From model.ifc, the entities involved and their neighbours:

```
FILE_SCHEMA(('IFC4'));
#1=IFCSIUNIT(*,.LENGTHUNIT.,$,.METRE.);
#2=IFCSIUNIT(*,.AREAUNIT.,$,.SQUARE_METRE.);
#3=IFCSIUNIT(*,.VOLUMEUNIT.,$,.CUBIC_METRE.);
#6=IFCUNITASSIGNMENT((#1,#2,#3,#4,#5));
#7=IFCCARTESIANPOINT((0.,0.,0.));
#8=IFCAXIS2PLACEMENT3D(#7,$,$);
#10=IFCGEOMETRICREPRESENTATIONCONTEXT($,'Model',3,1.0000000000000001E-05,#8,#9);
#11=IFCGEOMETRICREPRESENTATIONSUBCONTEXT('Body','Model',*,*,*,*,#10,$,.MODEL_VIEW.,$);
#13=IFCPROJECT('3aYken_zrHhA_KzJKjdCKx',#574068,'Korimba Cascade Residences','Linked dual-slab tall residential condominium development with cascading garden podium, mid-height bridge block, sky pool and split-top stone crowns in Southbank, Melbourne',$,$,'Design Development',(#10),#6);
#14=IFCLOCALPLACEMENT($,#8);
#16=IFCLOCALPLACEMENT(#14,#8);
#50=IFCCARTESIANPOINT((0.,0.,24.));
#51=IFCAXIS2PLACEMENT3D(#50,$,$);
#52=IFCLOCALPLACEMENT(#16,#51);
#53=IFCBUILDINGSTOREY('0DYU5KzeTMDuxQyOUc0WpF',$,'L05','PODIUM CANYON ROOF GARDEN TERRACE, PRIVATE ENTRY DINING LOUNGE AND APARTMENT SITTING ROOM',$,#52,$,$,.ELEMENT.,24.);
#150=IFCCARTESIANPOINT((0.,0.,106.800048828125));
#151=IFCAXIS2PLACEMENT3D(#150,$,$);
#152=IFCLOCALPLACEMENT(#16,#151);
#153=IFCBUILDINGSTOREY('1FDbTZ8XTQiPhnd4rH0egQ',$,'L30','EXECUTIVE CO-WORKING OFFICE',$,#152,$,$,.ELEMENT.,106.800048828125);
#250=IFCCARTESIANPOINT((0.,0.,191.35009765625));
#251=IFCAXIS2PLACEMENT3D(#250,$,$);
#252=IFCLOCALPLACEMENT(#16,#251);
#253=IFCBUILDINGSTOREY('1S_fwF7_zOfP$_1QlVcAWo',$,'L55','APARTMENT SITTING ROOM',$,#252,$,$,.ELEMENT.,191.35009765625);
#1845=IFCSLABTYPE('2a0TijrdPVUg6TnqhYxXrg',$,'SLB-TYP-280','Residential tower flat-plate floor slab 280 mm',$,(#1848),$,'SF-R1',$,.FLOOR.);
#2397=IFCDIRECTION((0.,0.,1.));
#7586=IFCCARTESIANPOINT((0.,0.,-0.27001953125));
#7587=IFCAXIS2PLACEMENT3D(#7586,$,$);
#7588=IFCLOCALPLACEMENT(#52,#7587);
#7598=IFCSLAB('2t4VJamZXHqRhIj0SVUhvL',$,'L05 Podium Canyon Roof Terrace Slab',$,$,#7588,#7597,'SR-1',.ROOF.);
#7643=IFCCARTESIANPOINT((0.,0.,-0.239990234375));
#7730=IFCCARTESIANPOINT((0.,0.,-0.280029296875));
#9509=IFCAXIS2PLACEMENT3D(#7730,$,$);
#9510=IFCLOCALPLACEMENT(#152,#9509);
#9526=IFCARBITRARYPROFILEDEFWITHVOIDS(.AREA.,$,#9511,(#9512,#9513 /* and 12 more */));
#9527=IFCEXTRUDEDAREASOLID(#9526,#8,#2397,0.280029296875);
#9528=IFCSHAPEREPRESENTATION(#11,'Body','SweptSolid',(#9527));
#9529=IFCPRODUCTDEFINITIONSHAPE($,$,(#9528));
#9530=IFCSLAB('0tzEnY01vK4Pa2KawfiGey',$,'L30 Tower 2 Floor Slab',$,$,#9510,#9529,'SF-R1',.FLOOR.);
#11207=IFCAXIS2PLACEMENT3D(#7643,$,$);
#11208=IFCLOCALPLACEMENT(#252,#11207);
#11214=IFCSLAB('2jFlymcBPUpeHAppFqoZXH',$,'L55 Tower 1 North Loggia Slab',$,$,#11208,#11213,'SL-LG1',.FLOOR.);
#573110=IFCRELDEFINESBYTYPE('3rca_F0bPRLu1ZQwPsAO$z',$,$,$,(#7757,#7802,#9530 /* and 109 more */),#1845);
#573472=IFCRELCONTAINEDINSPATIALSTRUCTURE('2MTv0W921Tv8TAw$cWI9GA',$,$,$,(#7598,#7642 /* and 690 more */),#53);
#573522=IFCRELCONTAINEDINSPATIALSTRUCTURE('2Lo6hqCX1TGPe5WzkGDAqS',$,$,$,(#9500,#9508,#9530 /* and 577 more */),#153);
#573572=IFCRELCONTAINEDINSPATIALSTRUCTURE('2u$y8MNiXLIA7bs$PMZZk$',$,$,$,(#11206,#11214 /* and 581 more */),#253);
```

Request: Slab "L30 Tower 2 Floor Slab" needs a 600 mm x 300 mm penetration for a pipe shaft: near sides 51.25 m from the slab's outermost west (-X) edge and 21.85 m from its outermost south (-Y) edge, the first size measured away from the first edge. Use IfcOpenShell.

```python
import numpy as np
import ifcopenshell
import ifcopenshell.api.feature
import ifcopenshell.api.geometry
import ifcopenshell.api.root
import ifcopenshell.geom
import ifcopenshell.util.placement
import ifcopenshell.util.representation
import ifcopenshell.util.shape
import ifcopenshell.util.unit

model = ifcopenshell.open("model.ifc")
unit_scale = ifcopenshell.util.unit.calculate_unit_scale(model)
settings = ifcopenshell.geom.settings()


def volume(element):
    """Net volume in cubic metres, openings subtracted."""
    shape = ifcopenshell.geom.create_shape(settings, element)
    return ifcopenshell.util.shape.get_volume(shape.geometry)


slab = model.by_guid("0tzEnY01vK4Pa2KawfiGey")
before = volume(slab)

# Extent in the slab's own axes, in metres. The edges named are its -X and -Y sides.
slab_shape = ifcopenshell.geom.create_shape(settings, slab)
vertices = ifcopenshell.util.shape.get_vertices(slab_shape.geometry)
x_min, y_min, bottom = vertices.min(axis=0)
top = vertices[:, 2].max()

opening = ifcopenshell.api.root.create_entity(model, ifc_class="IfcOpeningElement", name="Pipe shaft opening", predefined_type="OPENING")
context = ifcopenshell.util.representation.get_context(model, "Model", "Body", "MODEL_VIEW")
width, depth = 0.6, 0.3
outline = [(0.0, 0.0), (width, 0.0), (width, depth), (0.0, depth), (0.0, 0.0)]
# Overshoot both faces by 50 mm so the cut is clean.
shape = ifcopenshell.api.geometry.add_slab_representation(
    model, context=context, depth=top - bottom + 0.1, polyline=outline
)
ifcopenshell.api.geometry.assign_representation(model, product=opening, representation=shape)

matrix = ifcopenshell.util.placement.get_local_placement(slab.ObjectPlacement)
matrix[:, 3] = matrix @ np.append(np.array([x_min + 51.25, y_min + 21.85, bottom - 0.05]) / unit_scale, 1.0)
ifcopenshell.api.geometry.edit_object_placement(model, product=opening, matrix=matrix, is_si=False)
ifcopenshell.api.feature.add_feature(model, feature=opening, element=slab)

after = volume(slab)

print(f"slab volume {before:.3f} -> {after:.3f} m3")

model.write("model_rev.ifc")
```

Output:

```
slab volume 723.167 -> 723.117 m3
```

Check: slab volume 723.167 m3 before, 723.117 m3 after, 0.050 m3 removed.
